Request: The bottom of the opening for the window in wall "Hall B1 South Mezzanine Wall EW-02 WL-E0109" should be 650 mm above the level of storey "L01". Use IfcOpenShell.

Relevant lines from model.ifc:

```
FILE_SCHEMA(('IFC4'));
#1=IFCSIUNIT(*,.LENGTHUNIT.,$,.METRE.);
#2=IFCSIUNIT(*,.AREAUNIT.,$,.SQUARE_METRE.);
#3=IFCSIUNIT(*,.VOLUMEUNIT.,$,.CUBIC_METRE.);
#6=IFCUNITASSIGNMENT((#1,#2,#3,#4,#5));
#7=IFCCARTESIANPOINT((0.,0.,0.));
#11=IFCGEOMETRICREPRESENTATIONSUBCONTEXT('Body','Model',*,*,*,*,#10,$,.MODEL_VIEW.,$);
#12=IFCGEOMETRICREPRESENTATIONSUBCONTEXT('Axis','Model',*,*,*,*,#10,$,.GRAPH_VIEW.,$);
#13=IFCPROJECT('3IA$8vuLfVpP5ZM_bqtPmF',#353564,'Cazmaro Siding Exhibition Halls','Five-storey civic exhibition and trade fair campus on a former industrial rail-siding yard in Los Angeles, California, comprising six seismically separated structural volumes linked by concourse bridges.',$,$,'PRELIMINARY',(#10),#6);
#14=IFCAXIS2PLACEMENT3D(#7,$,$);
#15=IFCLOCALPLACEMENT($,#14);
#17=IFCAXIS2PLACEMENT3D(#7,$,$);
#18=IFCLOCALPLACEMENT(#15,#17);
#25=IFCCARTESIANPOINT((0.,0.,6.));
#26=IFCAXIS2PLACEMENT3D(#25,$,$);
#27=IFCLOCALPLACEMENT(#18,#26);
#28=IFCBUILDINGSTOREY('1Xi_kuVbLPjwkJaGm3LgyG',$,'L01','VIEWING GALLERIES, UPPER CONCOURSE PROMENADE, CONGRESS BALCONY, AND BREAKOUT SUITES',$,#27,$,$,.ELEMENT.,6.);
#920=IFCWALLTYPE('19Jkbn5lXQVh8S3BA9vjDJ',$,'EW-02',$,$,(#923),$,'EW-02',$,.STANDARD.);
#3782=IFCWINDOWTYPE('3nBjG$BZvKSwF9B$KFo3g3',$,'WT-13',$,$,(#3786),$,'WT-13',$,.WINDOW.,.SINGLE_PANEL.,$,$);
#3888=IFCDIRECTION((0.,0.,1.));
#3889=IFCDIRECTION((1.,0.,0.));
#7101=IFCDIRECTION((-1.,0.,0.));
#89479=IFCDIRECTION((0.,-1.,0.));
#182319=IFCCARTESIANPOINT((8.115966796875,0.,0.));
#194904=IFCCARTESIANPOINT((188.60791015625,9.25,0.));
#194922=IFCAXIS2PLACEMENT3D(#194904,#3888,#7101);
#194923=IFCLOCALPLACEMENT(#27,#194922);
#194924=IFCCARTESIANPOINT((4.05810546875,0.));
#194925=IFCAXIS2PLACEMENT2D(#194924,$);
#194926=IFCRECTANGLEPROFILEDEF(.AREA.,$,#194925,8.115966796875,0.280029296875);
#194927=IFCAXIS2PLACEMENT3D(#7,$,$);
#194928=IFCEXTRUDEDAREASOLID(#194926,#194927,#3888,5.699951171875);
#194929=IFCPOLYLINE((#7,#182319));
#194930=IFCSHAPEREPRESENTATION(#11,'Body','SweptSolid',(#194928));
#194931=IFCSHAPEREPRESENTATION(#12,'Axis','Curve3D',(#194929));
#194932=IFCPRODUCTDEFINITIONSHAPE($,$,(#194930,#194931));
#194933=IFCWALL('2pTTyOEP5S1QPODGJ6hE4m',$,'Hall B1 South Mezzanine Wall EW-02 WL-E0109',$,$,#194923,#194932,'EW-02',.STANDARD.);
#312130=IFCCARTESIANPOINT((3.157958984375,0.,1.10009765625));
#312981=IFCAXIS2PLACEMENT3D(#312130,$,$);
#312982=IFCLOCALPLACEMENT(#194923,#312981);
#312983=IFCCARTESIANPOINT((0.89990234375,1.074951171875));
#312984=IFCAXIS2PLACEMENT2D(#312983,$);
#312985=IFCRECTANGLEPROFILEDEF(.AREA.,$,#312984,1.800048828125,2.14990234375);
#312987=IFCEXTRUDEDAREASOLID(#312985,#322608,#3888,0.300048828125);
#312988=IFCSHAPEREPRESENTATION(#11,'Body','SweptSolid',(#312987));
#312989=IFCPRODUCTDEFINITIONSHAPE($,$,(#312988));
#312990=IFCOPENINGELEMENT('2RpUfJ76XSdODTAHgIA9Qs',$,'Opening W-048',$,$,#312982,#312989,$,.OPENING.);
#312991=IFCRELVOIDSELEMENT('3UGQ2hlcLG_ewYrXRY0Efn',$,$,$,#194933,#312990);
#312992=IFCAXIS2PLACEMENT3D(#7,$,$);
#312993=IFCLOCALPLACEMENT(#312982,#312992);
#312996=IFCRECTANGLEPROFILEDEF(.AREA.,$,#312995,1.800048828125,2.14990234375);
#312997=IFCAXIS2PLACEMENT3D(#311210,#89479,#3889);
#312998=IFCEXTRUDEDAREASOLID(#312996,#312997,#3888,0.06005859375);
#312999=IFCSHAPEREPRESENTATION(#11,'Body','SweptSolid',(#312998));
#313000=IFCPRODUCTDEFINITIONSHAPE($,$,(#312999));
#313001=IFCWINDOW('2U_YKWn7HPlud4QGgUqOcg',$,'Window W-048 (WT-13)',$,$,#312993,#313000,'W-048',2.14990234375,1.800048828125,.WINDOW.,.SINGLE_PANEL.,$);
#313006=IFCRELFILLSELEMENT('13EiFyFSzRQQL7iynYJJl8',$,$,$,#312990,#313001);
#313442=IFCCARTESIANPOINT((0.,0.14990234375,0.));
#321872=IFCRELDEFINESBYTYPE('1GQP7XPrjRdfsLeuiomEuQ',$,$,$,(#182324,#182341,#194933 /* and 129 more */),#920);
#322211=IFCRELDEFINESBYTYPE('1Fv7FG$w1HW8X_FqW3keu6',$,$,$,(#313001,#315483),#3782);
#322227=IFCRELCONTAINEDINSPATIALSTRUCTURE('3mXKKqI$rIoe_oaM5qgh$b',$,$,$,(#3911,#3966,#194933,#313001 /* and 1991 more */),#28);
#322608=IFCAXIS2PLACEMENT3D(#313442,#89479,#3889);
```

```python
import numpy as np
import ifcopenshell
import ifcopenshell.api.geometry
import ifcopenshell.geom
import ifcopenshell.util.element
import ifcopenshell.util.placement
import ifcopenshell.util.shape
import ifcopenshell.util.unit

model = ifcopenshell.open("model.ifc")
unit_scale = ifcopenshell.util.unit.calculate_unit_scale(model)

window = model.by_guid("2U_YKWn7HPlud4QGgUqOcg")
opening = window.FillsVoids[0].RelatingOpeningElement
storey = ifcopenshell.util.element.get_container(window, ifc_class="IfcBuildingStorey")
level = ifcopenshell.util.placement.get_local_placement(storey.ObjectPlacement)[2, 3]

# The opening's origin need not be at the sill, so measure its lowest point.
shape = ifcopenshell.geom.create_shape(ifcopenshell.geom.settings(), opening)
bottom = ifcopenshell.util.shape.get_shape_bottom_elevation(shape, shape.geometry) / unit_scale
dz = level + 0.65 / unit_scale - bottom

shift = np.array([0.0, 0.0, dz])
# The window is placed relative to its opening, so it follows when the opening moves.
matrix = ifcopenshell.util.placement.get_local_placement(opening.ObjectPlacement)
matrix[:3, 3] += shift
ifcopenshell.api.geometry.edit_object_placement(
    model, product=opening, matrix=matrix, is_si=False, should_transform_children=True
)

print(f"moved by {dz * unit_scale:+.3f} m")

model.write("model_v2.ifc")
```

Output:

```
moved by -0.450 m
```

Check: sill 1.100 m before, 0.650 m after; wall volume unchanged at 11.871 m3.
